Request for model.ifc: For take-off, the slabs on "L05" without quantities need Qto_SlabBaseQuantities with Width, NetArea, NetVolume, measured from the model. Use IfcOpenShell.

First a look at what the model holds.

```python
import ifcopenshell
import ifcopenshell.util.element
import ifcopenshell.util.unit

model = ifcopenshell.open("model.ifc")
print(model.schema)
for unit_type in ("LENGTHUNIT", "AREAUNIT", "VOLUMEUNIT"):
    print(unit_type, ifcopenshell.util.unit.calculate_unit_scale(model, unit_type))
storey = next(s for s in model.by_type("IfcBuildingStorey") if s.Name == "L05")
slabs = [e for e in ifcopenshell.util.element.get_decomposition(storey) if e.is_a("IfcSlab")]
for e in sorted(slabs, key=lambda e: e.id()):
    print(e.id(), e.is_a(), e.Name, list(ifcopenshell.util.element.get_psets(e, qtos_only=True)), sep=" | ")
```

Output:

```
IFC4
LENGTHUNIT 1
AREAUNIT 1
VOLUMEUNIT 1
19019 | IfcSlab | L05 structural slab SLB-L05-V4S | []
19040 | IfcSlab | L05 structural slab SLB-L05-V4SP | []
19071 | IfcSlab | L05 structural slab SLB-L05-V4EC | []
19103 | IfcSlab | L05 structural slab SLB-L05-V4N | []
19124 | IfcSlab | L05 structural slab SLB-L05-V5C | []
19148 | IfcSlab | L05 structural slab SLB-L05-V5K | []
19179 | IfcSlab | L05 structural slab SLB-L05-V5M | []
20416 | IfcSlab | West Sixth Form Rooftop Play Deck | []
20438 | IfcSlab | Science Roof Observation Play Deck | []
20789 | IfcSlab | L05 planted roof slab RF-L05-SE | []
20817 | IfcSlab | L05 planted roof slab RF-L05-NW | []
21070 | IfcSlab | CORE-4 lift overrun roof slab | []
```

```python
import ifcopenshell
import ifcopenshell.api.pset
import ifcopenshell.geom
import ifcopenshell.util.element
import ifcopenshell.util.shape
import ifcopenshell.util.unit

model = ifcopenshell.open("model.ifc")
unit_scale = ifcopenshell.util.unit.calculate_unit_scale(model)
area_scale = ifcopenshell.util.unit.calculate_unit_scale(model, "AREAUNIT")
volume_scale = ifcopenshell.util.unit.calculate_unit_scale(model, "VOLUMEUNIT")
settings = ifcopenshell.geom.settings()

storey = next(s for s in model.by_type("IfcBuildingStorey") if s.Name == "L05")
slabs = [e for e in ifcopenshell.util.element.get_decomposition(storey) if e.is_a("IfcSlab")]

for e in sorted(slabs, key=lambda e: e.id()):
    if ifcopenshell.util.element.get_psets(e, qtos_only=True, should_inherit=False):
        continue
    # Geometry comes back in metres, in the element's own axes.
    shape = ifcopenshell.geom.create_shape(settings, e)
    values = {
        "Width": ifcopenshell.util.shape.get_z(shape.geometry) / unit_scale,
        "NetArea": ifcopenshell.util.shape.get_footprint_area(shape.geometry) / area_scale,
        "NetVolume": ifcopenshell.util.shape.get_volume(shape.geometry) / volume_scale,
    }
    qto = ifcopenshell.api.pset.add_qto(model, product=e, name="Qto_SlabBaseQuantities")
    ifcopenshell.api.pset.edit_qto(model, qto=qto, properties=values)
    print(e.id(), {k: round(v, 3) for k, v in values.items()})

model.write("model_v2.ifc")
```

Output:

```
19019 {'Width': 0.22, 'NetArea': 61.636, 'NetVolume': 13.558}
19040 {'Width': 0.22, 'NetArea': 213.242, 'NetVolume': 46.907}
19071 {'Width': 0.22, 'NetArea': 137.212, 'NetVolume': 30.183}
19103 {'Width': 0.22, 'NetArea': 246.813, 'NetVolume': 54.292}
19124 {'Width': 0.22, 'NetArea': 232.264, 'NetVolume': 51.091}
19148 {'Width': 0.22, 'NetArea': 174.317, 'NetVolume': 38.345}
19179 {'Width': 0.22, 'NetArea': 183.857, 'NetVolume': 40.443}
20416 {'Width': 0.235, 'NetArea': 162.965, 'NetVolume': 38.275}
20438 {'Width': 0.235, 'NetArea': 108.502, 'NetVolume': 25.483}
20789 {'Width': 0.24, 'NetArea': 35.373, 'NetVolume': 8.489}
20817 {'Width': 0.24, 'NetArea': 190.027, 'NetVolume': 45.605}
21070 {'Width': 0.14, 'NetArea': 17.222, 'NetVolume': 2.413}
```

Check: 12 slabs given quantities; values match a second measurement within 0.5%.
